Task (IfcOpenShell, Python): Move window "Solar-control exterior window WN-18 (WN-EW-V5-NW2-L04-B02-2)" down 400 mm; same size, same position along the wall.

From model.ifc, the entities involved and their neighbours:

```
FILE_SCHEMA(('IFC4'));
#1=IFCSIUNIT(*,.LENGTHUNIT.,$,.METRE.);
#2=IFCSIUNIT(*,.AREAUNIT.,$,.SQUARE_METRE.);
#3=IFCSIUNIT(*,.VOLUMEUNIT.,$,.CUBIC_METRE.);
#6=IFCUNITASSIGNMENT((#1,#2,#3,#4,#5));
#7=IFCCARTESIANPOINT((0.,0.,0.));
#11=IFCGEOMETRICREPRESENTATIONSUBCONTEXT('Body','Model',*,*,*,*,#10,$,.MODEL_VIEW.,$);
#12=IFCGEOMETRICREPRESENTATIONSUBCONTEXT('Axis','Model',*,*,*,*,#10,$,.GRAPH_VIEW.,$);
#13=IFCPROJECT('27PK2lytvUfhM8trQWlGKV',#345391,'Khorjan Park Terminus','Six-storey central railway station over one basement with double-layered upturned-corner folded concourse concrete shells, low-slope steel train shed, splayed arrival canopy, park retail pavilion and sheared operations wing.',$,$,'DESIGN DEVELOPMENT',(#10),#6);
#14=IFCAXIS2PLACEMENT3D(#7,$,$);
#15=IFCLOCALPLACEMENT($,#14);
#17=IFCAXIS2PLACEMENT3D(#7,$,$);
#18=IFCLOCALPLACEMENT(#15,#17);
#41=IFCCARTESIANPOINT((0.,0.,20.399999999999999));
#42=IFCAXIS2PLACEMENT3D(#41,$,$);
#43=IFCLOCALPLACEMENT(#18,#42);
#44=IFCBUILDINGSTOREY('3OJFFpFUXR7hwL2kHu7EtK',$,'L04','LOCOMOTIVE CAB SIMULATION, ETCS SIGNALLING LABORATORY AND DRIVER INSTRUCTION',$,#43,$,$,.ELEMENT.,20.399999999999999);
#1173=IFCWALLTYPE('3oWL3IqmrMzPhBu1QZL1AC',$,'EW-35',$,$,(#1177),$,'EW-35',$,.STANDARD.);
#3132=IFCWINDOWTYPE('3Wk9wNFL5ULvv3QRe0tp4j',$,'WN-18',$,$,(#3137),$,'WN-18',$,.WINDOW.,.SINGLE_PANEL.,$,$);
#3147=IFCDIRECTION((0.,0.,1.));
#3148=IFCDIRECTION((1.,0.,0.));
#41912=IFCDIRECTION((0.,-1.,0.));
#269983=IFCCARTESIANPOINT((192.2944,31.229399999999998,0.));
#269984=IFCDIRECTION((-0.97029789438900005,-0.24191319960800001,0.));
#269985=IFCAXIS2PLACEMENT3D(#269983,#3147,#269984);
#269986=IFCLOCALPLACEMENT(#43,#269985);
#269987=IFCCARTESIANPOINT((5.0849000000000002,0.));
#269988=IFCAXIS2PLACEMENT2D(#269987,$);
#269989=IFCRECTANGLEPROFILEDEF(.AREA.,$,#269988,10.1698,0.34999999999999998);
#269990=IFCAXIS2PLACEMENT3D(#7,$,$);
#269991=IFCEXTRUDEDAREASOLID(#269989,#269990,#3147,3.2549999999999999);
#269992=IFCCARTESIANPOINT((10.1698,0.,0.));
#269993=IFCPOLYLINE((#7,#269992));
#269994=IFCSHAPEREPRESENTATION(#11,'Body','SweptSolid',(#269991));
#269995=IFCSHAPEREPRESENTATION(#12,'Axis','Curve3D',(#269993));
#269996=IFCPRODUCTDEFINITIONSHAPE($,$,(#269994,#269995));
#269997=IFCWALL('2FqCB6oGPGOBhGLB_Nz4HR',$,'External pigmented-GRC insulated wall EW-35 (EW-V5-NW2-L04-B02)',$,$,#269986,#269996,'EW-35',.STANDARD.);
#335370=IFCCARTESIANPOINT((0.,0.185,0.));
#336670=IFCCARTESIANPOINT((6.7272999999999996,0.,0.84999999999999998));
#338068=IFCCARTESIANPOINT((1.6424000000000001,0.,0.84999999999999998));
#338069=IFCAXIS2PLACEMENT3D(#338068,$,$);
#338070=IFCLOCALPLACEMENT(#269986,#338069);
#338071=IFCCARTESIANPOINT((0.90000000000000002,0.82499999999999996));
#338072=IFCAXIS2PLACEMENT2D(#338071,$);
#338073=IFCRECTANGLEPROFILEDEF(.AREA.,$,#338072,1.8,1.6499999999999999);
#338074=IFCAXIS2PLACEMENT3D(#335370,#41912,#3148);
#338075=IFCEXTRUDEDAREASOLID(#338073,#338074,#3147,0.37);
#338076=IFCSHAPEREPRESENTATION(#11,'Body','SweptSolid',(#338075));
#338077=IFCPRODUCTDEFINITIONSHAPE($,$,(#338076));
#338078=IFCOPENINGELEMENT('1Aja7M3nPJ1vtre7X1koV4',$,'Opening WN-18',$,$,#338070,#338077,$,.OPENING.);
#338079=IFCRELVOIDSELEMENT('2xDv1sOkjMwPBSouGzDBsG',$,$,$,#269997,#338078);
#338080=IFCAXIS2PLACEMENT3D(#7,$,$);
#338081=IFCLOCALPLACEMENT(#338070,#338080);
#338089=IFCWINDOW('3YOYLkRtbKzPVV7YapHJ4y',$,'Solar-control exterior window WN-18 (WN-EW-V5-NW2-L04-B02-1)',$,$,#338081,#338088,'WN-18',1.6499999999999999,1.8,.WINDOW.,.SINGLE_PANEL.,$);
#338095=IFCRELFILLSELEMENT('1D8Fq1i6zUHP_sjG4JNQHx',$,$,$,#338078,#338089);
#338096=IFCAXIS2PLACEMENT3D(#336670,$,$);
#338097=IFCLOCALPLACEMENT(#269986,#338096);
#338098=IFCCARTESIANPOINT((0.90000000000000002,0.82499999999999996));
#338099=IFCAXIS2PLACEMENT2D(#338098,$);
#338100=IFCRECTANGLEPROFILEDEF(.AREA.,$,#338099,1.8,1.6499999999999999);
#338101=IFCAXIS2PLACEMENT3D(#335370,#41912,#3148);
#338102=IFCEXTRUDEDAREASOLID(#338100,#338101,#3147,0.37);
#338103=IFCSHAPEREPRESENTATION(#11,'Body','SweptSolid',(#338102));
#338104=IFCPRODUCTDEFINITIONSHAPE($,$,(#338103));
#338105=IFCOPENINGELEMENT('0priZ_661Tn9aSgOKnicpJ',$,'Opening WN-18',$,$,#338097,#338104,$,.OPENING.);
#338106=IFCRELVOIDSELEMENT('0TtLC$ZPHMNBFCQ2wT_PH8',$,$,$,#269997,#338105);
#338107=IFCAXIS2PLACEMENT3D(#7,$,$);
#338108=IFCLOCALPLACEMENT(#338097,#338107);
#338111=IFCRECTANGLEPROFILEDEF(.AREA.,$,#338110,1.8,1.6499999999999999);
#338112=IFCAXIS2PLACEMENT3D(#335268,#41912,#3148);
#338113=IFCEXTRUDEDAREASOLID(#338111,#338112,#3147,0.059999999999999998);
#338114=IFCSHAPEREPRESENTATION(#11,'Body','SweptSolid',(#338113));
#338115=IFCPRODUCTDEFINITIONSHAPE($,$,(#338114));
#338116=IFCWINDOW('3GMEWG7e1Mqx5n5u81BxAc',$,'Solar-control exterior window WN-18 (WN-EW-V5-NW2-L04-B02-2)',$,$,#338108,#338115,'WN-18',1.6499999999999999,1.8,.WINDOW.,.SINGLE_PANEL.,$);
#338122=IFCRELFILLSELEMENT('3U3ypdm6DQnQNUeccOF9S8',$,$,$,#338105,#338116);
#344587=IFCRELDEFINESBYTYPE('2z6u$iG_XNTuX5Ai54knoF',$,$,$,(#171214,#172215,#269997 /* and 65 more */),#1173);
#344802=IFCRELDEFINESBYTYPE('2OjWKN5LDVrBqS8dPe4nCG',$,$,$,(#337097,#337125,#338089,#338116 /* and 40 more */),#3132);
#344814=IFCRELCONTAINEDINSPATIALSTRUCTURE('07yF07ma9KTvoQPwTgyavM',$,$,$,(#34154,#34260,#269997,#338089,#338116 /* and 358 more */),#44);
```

```python
import numpy as np
import ifcopenshell
import ifcopenshell.api.geometry
import ifcopenshell.util.placement
import ifcopenshell.util.unit

model = ifcopenshell.open("model.ifc")
unit_scale = ifcopenshell.util.unit.calculate_unit_scale(model)

window = model.by_guid("3GMEWG7e1Mqx5n5u81BxAc")
opening = window.FillsVoids[0].RelatingOpeningElement
dz = -0.4

shift = np.array([0.0, 0.0, dz])
# The window is placed relative to its opening, so it follows when the opening moves.
matrix = ifcopenshell.util.placement.get_local_placement(opening.ObjectPlacement)
matrix[:3, 3] += shift
ifcopenshell.api.geometry.edit_object_placement(
    model, product=opening, matrix=matrix, is_si=False, should_transform_children=True
)

print(f"moved by {dz * unit_scale:+.3f} m")

model.write("model_rev.ifc")
```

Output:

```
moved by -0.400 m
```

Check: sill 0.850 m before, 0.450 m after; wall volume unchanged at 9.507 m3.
